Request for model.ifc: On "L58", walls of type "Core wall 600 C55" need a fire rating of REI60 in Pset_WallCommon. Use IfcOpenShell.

First a look at what the model holds.

```python
import ifcopenshell
import ifcopenshell.util.element

model = ifcopenshell.open("model.ifc")
print(model.schema)
storey = next(s for s in model.by_type("IfcBuildingStorey") if s.Name == "L58")
walls = [e for e in ifcopenshell.util.element.get_decomposition(storey) if e.is_a("IfcWall")]
seen = {}
for e in walls:
    element_type = ifcopenshell.util.element.get_type(e)
    key = (element_type.Name if element_type != e and element_type else None, ifcopenshell.util.element.get_pset(e, "Pset_WallCommon", "FireRating"))
    seen[key] = seen.get(key, 0) + 1
for (name, value), count in sorted(seen.items(), key=str):
    print(count, "x", name, "|", value)
```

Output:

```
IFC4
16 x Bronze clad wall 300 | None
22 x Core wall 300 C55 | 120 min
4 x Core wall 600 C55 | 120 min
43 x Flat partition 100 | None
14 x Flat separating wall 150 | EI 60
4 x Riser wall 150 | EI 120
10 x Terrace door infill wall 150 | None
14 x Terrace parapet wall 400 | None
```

```python
import ifcopenshell
import ifcopenshell.api.pset
import ifcopenshell.util.element

model = ifcopenshell.open("model.ifc")

storey = next(s for s in model.by_type("IfcBuildingStorey") if s.Name == "L58")
walls = [e for e in ifcopenshell.util.element.get_decomposition(storey) if e.is_a("IfcWall")]

count = 0
for e in walls:
    element_type = ifcopenshell.util.element.get_type(e)
    if element_type in (None, e) or element_type.Name != "Core wall 600 C55":
        continue
    found = ifcopenshell.util.element.get_pset(e, "Pset_WallCommon", should_inherit=False)
    if found:
        pset = model.by_id(found["id"])
        if len(ifcopenshell.util.element.get_elements_by_pset(pset)) > 1:
            pset = ifcopenshell.api.pset.unshare_pset(model, products=[e], pset=pset)[0]
    else:
        pset = ifcopenshell.api.pset.add_pset(model, product=e, name="Pset_WallCommon")
    ifcopenshell.api.pset.edit_pset(model, pset=pset, properties={"FireRating": "REI60"})
    count += 1

print(count, "walls updated")

model.write("model_rev.ifc")
```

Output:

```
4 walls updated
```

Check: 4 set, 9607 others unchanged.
